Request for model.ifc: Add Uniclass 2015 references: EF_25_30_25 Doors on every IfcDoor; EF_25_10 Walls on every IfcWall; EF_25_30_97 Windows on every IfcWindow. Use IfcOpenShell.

First a look at what the model holds.

```python
import ifcopenshell

model = ifcopenshell.open("model.ifc")
print(model.schema)
print("classifications:", [c.Name for c in model.by_type("IfcClassification")])
for ifc_class in ("IfcDoor", "IfcRoof", "IfcStair", "IfcWall", "IfcWindow"):
    print(ifc_class, len(model.by_type(ifc_class)))
```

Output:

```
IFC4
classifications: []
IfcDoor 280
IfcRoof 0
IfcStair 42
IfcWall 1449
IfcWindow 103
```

```python
import ifcopenshell
import ifcopenshell.api.classification

model = ifcopenshell.open("model.ifc")

system = ifcopenshell.api.classification.add_classification(model, classification="Uniclass 2015")

codes = {
    "IfcDoor": ("EF_25_30_25", "Doors"),
    "IfcWall": ("EF_25_10", "Walls"),
    "IfcWindow": ("EF_25_30_97", "Windows"),
}
for ifc_class, (code, name) in codes.items():
    products = model.by_type(ifc_class)
    ifcopenshell.api.classification.add_reference(
        model, products=products, classification=system, identification=code, name=name
    )
    print(code, len(products))

model.write("model-out.ifc")
```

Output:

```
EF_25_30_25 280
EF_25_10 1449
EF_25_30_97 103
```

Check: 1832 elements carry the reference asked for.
